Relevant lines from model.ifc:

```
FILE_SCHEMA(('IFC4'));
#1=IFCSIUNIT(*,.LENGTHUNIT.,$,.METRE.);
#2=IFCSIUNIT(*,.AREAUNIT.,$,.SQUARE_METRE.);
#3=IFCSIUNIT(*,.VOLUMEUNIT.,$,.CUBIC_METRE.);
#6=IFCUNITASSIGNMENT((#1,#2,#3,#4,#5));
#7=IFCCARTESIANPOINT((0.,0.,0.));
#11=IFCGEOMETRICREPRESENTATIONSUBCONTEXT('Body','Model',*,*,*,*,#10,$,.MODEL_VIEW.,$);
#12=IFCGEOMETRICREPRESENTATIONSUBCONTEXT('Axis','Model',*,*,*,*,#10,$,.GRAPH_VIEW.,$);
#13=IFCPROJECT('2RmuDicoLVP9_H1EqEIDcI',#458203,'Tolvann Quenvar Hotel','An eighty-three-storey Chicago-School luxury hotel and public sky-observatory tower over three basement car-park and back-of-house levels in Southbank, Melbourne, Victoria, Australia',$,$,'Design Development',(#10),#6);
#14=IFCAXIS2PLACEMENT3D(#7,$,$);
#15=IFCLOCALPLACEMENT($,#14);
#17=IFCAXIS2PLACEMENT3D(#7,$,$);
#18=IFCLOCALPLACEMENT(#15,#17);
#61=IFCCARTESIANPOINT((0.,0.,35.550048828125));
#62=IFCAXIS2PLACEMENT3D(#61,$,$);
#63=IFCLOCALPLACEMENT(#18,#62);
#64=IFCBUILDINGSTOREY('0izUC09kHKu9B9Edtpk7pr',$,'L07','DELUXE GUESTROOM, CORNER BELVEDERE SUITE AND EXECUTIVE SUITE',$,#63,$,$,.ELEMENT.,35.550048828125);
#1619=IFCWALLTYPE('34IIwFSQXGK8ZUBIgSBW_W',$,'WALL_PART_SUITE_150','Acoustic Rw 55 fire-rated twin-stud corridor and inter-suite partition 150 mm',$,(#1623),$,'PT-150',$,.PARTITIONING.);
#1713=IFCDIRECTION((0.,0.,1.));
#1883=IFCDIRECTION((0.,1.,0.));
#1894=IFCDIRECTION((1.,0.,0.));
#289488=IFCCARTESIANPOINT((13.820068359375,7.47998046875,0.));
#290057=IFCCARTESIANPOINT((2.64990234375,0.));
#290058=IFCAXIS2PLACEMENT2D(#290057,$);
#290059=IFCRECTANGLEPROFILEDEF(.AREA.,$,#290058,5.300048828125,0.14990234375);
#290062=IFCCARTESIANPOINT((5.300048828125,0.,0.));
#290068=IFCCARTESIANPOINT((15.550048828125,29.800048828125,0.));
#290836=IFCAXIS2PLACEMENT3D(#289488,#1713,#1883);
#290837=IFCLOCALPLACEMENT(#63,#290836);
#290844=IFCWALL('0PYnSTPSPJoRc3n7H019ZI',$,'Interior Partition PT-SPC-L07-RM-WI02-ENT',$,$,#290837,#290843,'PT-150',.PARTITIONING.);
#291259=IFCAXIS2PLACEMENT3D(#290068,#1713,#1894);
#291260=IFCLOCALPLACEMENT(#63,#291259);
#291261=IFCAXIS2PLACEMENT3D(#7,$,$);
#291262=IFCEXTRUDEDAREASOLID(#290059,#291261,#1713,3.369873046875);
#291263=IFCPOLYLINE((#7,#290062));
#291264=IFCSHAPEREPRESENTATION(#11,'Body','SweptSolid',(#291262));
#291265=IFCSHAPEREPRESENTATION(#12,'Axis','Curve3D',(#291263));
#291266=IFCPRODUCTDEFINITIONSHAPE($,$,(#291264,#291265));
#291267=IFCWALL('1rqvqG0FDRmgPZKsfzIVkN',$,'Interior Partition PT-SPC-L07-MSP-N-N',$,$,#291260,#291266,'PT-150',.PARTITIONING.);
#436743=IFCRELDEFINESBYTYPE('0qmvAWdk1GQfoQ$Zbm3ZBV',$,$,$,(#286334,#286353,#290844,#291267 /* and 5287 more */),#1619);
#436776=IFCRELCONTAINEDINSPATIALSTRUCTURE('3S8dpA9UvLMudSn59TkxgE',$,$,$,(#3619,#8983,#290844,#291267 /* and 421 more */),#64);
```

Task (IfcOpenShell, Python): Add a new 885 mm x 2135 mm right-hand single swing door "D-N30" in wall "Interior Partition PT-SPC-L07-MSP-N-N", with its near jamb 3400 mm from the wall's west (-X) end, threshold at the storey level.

```python
import numpy as np
import ifcopenshell
import ifcopenshell.api.feature
import ifcopenshell.api.geometry
import ifcopenshell.api.root
import ifcopenshell.api.spatial
import ifcopenshell.geom
import ifcopenshell.util.element
import ifcopenshell.util.placement
import ifcopenshell.util.representation
import ifcopenshell.util.shape
import ifcopenshell.util.unit

model = ifcopenshell.open("model.ifc")
unit_scale = ifcopenshell.util.unit.calculate_unit_scale(model)
settings = ifcopenshell.geom.settings()


def volume(element):
    """Net volume in cubic metres, openings subtracted."""
    shape = ifcopenshell.geom.create_shape(settings, element)
    return ifcopenshell.util.shape.get_volume(shape.geometry)


wall = model.by_id(291267)
storey = ifcopenshell.util.element.get_container(wall, ifc_class="IfcBuildingStorey")
context = ifcopenshell.util.representation.get_context(model, "Model", "Body", "MODEL_VIEW")
before = volume(wall)

width, height, from_end, sill = 0.885, 2.135, 3.4, 0.0  # metres

# The wall runs along its own X axis, and the end named is its -X end.
wall_shape = ifcopenshell.geom.create_shape(settings, wall)
x, y, z = ifcopenshell.util.shape.get_vertices(wall_shape.geometry).T
start = x.min() + from_end
face, thickness = float(y.min()), float(y.max() - y.min())
wall_matrix = ifcopenshell.util.placement.get_local_placement(wall.ObjectPlacement)
level = ifcopenshell.util.placement.get_local_placement(storey.ObjectPlacement)[2, 3]


def in_wall(x, y):
    """Placement at x, y metres in the wall's axes, at sill height."""
    matrix = wall_matrix.copy()
    matrix[:, 3] = wall_matrix @ np.array([x / unit_scale, y / unit_scale, 0.0, 1.0])
    matrix[2, 3] = level + sill / unit_scale
    return matrix


# Opening: a box that overshoots both wall faces by 50 mm.
opening = ifcopenshell.api.root.create_entity(model, ifc_class="IfcOpeningElement", predefined_type="OPENING")
box = ifcopenshell.api.geometry.add_wall_representation(
    model, context=context, length=width, height=height, thickness=thickness + 0.1
)
ifcopenshell.api.geometry.assign_representation(model, product=opening, representation=box)
ifcopenshell.api.geometry.edit_object_placement(model, product=opening, matrix=in_wall(start, face - 0.05), is_si=False)
ifcopenshell.api.feature.add_feature(model, feature=opening, element=wall)

door = ifcopenshell.api.root.create_entity(model, ifc_class="IfcDoor", name="D-N30", predefined_type="DOOR")
door.OverallWidth, door.OverallHeight = width / unit_scale, height / unit_scale
door.OperationType = "SINGLE_SWING_RIGHT"
body = ifcopenshell.api.geometry.add_door_representation(
    model,
    context=context,
    overall_width=door.OverallWidth,
    overall_height=door.OverallHeight,
    operation_type="SINGLE_SWING_RIGHT",
    lining_properties={"LiningDepth": thickness / unit_scale, "ThresholdDepth": thickness / unit_scale},
)
ifcopenshell.api.geometry.assign_representation(model, product=door, representation=body)
ifcopenshell.api.spatial.assign_container(model, products=[door], relating_structure=storey)
ifcopenshell.api.feature.add_filling(model, opening=opening, element=door)

# The lining spans the wall, so the door starts at the wall face.
ifcopenshell.api.geometry.edit_object_placement(model, product=door, matrix=in_wall(start, face), is_si=False)

after = volume(wall)

print(f"wall volume {before:.3f} -> {after:.3f} m3")

model.write("model_edited.ifc")
```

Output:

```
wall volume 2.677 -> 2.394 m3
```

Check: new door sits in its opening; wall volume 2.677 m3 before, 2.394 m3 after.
